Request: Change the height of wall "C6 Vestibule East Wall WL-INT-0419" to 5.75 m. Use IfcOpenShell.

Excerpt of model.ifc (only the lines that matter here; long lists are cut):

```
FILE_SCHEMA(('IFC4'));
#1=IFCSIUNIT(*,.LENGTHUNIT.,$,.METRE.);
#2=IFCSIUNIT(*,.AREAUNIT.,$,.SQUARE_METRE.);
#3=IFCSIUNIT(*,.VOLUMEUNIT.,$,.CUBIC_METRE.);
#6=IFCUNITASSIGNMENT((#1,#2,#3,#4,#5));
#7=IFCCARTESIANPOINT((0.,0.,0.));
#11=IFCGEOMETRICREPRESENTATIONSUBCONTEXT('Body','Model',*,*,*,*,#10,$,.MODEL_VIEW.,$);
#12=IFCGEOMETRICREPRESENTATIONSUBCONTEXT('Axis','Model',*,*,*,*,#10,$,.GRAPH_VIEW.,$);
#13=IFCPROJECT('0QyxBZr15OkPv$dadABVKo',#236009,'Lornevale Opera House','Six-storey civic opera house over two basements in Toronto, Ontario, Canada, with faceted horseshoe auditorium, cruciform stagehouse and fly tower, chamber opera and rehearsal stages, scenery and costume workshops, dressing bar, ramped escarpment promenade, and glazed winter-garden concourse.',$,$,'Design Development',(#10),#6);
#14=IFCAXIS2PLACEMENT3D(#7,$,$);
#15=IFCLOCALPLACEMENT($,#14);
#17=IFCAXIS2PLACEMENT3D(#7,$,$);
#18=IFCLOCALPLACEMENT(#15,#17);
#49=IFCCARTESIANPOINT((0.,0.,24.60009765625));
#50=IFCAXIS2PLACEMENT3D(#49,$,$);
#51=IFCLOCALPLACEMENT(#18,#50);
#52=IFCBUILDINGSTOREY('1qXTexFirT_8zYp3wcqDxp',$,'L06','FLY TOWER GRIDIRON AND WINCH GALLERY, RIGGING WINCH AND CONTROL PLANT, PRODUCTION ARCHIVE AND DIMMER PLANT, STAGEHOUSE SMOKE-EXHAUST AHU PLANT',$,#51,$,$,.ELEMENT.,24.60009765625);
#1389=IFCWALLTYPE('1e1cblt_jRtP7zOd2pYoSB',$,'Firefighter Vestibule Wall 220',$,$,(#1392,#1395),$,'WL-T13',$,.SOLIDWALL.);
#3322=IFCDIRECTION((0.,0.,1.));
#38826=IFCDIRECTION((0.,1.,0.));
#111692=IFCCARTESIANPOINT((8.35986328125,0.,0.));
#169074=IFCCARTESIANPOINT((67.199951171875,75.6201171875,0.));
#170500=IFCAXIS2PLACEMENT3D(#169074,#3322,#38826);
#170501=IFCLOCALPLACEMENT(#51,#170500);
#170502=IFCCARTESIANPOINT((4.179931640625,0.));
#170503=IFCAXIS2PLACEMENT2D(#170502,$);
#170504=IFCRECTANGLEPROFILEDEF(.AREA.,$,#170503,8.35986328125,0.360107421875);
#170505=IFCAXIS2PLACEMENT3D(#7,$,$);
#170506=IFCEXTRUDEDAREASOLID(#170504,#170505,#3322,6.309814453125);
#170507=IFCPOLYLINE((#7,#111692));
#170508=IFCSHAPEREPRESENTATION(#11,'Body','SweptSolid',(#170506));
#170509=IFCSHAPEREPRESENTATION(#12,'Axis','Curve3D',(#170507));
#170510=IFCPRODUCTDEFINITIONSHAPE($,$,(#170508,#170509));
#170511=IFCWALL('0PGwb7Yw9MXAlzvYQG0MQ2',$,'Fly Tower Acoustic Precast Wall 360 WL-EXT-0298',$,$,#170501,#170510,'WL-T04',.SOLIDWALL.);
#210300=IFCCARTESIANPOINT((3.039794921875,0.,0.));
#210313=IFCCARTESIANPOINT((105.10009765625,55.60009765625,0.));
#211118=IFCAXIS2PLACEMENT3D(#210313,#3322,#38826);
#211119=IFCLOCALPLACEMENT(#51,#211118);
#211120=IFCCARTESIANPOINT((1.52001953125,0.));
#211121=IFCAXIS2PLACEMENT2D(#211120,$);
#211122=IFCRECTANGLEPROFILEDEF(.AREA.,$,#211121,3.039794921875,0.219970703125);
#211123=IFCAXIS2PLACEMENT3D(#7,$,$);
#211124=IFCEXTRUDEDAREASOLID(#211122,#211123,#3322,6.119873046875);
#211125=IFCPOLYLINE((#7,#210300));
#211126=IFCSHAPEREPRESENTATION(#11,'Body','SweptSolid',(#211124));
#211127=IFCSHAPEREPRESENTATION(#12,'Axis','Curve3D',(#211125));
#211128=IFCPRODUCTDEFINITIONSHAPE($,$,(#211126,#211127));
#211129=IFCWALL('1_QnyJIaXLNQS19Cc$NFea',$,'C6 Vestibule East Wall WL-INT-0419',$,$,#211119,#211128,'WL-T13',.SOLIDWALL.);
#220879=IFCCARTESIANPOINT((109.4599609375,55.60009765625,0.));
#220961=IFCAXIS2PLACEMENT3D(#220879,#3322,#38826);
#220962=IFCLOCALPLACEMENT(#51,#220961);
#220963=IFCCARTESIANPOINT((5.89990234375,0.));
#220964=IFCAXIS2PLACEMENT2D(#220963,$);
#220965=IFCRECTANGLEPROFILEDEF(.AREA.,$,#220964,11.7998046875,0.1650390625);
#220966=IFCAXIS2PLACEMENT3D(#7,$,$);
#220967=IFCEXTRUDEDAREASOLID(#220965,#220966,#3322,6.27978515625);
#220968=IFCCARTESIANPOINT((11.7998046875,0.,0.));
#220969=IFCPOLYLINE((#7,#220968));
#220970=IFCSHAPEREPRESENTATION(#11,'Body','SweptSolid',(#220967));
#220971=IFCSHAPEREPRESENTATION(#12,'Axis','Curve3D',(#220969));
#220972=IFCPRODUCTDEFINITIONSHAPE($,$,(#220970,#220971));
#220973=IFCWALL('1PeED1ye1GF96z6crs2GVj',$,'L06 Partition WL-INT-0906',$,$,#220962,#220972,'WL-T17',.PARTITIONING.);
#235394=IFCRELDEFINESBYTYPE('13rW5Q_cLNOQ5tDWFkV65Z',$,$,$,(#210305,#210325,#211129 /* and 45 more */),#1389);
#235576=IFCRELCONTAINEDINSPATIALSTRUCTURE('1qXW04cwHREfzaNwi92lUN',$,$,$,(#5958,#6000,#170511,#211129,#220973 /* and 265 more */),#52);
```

```python
import ifcopenshell
import ifcopenshell.geom
import ifcopenshell.util.representation
import ifcopenshell.util.shape

model = ifcopenshell.open("model.ifc")
settings = ifcopenshell.geom.settings()


def volume(element):
    """Net volume in cubic metres, openings subtracted."""
    shape = ifcopenshell.geom.create_shape(settings, element)
    return ifcopenshell.util.shape.get_volume(shape.geometry)


wall = model.by_guid("1_QnyJIaXLNQS19Cc$NFea")
before = volume(wall)

body = ifcopenshell.util.representation.get_representation(wall, "Model", "Body")
solid = body.Items[0]
old_height = solid.Depth
solid.Depth = 5.75
after = volume(wall)

print(f"height {old_height:g} -> {solid.Depth:g}, volume {before:.3f} -> {after:.3f} m3")

model.write("model-out.ifc")
```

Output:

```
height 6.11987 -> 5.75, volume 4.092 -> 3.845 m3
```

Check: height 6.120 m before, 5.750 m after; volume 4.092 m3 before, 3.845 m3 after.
